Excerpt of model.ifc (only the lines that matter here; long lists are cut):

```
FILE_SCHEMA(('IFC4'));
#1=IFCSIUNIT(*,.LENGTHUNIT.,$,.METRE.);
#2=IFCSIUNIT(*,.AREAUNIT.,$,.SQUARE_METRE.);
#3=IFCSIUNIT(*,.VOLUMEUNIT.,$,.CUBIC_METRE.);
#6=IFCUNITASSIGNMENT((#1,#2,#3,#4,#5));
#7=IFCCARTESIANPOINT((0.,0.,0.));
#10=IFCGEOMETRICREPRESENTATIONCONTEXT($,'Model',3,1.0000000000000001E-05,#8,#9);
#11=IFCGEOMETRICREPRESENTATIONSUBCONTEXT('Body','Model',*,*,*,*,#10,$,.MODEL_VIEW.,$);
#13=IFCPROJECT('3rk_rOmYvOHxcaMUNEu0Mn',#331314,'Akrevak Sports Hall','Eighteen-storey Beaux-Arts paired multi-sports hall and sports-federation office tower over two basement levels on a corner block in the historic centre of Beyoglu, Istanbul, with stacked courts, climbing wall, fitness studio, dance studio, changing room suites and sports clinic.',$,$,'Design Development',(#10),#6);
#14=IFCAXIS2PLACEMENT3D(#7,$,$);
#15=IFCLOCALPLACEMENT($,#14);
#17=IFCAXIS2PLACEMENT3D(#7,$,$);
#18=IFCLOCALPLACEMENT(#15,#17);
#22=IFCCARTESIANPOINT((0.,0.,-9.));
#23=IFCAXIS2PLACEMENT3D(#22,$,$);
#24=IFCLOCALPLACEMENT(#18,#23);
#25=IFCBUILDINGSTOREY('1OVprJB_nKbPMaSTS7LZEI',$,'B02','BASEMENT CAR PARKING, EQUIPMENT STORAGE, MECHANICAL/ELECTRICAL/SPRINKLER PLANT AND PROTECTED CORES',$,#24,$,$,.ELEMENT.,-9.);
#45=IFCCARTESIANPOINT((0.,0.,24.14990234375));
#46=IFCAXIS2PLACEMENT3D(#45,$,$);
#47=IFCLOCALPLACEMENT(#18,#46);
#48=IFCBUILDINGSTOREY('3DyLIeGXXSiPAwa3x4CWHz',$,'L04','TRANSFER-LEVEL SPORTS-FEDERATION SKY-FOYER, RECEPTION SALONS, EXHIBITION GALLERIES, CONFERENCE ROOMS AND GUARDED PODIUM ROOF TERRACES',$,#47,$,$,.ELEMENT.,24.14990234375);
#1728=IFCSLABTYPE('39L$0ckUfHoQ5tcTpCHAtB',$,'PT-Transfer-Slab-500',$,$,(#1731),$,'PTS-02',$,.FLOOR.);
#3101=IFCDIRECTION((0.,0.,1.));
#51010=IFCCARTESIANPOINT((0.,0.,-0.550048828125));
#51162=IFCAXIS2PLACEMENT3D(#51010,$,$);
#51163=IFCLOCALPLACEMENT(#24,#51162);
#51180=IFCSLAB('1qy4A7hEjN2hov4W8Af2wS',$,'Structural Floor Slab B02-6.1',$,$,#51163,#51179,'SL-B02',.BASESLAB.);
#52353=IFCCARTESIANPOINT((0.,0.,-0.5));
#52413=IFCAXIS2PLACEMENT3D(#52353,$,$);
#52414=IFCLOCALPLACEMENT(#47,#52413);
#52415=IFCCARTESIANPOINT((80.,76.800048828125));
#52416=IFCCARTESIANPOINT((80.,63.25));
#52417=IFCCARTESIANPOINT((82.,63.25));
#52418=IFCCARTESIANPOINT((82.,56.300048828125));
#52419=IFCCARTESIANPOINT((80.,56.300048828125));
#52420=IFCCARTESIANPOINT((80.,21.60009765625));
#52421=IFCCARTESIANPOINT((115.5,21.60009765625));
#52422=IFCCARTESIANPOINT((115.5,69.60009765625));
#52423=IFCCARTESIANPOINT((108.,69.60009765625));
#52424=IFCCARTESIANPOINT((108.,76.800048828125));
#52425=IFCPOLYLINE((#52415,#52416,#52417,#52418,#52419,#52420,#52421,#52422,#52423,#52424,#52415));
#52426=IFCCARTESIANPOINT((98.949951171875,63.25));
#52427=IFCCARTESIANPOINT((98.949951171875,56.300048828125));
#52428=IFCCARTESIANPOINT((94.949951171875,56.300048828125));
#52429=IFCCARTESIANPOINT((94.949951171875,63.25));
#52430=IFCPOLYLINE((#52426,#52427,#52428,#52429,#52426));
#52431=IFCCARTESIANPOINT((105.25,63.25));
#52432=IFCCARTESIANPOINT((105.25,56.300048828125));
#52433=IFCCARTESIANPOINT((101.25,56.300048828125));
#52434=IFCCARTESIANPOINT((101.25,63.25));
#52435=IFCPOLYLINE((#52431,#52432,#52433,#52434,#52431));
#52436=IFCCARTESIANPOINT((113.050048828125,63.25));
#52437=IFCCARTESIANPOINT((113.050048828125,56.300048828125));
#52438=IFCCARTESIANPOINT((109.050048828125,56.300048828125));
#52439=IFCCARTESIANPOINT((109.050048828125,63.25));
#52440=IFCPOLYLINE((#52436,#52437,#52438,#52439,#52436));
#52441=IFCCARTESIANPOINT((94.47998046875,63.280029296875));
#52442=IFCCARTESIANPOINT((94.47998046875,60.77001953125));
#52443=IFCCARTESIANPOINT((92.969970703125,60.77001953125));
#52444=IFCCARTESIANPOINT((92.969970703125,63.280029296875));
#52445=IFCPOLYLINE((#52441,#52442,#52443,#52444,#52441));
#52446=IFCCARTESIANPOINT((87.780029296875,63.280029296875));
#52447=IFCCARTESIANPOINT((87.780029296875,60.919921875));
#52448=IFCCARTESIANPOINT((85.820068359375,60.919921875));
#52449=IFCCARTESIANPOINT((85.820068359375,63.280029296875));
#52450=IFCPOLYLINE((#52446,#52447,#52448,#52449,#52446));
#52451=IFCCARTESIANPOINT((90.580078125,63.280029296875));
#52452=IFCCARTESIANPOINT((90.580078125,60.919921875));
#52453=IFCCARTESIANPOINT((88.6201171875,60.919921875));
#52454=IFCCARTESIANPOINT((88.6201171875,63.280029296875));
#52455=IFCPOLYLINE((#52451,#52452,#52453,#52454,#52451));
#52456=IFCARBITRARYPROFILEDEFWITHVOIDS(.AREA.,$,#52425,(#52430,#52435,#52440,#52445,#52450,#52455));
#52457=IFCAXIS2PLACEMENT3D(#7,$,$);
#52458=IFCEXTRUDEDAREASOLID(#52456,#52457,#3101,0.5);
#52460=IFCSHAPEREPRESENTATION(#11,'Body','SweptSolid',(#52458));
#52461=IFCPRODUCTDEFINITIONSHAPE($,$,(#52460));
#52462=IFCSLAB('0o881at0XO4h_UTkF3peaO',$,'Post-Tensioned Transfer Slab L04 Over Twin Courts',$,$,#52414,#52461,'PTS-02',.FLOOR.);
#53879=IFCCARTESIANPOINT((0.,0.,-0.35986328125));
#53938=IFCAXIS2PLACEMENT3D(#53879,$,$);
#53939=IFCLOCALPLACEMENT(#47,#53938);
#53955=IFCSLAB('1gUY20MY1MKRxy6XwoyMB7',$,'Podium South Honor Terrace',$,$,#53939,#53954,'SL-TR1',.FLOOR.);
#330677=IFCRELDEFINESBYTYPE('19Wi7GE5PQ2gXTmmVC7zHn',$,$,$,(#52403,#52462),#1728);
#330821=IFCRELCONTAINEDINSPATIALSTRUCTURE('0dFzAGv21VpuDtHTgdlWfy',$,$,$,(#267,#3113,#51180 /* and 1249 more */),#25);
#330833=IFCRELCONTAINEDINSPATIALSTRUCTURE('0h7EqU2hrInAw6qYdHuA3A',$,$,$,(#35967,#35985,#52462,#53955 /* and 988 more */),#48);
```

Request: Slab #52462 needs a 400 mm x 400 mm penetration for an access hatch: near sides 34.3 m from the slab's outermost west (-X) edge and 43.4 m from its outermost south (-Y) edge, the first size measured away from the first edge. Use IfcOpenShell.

```python
import numpy as np
import ifcopenshell
import ifcopenshell.api.feature
import ifcopenshell.api.geometry
import ifcopenshell.api.root
import ifcopenshell.geom
import ifcopenshell.util.placement
import ifcopenshell.util.representation
import ifcopenshell.util.shape
import ifcopenshell.util.unit

model = ifcopenshell.open("model.ifc")
unit_scale = ifcopenshell.util.unit.calculate_unit_scale(model)
settings = ifcopenshell.geom.settings()


def volume(element):
    """Net volume in cubic metres, openings subtracted."""
    shape = ifcopenshell.geom.create_shape(settings, element)
    return ifcopenshell.util.shape.get_volume(shape.geometry)


slab = model.by_id(52462)
before = volume(slab)

# Extent in the slab's own axes, in metres. The edges named are its -X and -Y sides.
slab_shape = ifcopenshell.geom.create_shape(settings, slab)
vertices = ifcopenshell.util.shape.get_vertices(slab_shape.geometry)
x_min, y_min, bottom = vertices.min(axis=0)
top = vertices[:, 2].max()

opening = ifcopenshell.api.root.create_entity(model, ifc_class="IfcOpeningElement", name="Access hatch opening", predefined_type="OPENING")
context = ifcopenshell.util.representation.get_context(model, "Model", "Body", "MODEL_VIEW")
width, depth = 0.4, 0.4
outline = [(0.0, 0.0), (width, 0.0), (width, depth), (0.0, depth), (0.0, 0.0)]
# Overshoot both faces by 50 mm so the cut is clean.
shape = ifcopenshell.api.geometry.add_slab_representation(
    model, context=context, depth=top - bottom + 0.1, polyline=outline
)
ifcopenshell.api.geometry.assign_representation(model, product=opening, representation=shape)

matrix = ifcopenshell.util.placement.get_local_placement(slab.ObjectPlacement)
matrix[:, 3] = matrix @ np.append(np.array([x_min + 34.3, y_min + 43.4, bottom - 0.05]) / unit_scale, 1.0)
ifcopenshell.api.geometry.edit_object_placement(model, product=opening, matrix=matrix, is_si=False)
ifcopenshell.api.feature.add_feature(model, feature=opening, element=slab)

after = volume(slab)

print(f"slab volume {before:.3f} -> {after:.3f} m3")

model.write("model-out.ifc")
```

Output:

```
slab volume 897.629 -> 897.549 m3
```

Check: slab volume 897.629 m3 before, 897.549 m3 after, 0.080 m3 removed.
